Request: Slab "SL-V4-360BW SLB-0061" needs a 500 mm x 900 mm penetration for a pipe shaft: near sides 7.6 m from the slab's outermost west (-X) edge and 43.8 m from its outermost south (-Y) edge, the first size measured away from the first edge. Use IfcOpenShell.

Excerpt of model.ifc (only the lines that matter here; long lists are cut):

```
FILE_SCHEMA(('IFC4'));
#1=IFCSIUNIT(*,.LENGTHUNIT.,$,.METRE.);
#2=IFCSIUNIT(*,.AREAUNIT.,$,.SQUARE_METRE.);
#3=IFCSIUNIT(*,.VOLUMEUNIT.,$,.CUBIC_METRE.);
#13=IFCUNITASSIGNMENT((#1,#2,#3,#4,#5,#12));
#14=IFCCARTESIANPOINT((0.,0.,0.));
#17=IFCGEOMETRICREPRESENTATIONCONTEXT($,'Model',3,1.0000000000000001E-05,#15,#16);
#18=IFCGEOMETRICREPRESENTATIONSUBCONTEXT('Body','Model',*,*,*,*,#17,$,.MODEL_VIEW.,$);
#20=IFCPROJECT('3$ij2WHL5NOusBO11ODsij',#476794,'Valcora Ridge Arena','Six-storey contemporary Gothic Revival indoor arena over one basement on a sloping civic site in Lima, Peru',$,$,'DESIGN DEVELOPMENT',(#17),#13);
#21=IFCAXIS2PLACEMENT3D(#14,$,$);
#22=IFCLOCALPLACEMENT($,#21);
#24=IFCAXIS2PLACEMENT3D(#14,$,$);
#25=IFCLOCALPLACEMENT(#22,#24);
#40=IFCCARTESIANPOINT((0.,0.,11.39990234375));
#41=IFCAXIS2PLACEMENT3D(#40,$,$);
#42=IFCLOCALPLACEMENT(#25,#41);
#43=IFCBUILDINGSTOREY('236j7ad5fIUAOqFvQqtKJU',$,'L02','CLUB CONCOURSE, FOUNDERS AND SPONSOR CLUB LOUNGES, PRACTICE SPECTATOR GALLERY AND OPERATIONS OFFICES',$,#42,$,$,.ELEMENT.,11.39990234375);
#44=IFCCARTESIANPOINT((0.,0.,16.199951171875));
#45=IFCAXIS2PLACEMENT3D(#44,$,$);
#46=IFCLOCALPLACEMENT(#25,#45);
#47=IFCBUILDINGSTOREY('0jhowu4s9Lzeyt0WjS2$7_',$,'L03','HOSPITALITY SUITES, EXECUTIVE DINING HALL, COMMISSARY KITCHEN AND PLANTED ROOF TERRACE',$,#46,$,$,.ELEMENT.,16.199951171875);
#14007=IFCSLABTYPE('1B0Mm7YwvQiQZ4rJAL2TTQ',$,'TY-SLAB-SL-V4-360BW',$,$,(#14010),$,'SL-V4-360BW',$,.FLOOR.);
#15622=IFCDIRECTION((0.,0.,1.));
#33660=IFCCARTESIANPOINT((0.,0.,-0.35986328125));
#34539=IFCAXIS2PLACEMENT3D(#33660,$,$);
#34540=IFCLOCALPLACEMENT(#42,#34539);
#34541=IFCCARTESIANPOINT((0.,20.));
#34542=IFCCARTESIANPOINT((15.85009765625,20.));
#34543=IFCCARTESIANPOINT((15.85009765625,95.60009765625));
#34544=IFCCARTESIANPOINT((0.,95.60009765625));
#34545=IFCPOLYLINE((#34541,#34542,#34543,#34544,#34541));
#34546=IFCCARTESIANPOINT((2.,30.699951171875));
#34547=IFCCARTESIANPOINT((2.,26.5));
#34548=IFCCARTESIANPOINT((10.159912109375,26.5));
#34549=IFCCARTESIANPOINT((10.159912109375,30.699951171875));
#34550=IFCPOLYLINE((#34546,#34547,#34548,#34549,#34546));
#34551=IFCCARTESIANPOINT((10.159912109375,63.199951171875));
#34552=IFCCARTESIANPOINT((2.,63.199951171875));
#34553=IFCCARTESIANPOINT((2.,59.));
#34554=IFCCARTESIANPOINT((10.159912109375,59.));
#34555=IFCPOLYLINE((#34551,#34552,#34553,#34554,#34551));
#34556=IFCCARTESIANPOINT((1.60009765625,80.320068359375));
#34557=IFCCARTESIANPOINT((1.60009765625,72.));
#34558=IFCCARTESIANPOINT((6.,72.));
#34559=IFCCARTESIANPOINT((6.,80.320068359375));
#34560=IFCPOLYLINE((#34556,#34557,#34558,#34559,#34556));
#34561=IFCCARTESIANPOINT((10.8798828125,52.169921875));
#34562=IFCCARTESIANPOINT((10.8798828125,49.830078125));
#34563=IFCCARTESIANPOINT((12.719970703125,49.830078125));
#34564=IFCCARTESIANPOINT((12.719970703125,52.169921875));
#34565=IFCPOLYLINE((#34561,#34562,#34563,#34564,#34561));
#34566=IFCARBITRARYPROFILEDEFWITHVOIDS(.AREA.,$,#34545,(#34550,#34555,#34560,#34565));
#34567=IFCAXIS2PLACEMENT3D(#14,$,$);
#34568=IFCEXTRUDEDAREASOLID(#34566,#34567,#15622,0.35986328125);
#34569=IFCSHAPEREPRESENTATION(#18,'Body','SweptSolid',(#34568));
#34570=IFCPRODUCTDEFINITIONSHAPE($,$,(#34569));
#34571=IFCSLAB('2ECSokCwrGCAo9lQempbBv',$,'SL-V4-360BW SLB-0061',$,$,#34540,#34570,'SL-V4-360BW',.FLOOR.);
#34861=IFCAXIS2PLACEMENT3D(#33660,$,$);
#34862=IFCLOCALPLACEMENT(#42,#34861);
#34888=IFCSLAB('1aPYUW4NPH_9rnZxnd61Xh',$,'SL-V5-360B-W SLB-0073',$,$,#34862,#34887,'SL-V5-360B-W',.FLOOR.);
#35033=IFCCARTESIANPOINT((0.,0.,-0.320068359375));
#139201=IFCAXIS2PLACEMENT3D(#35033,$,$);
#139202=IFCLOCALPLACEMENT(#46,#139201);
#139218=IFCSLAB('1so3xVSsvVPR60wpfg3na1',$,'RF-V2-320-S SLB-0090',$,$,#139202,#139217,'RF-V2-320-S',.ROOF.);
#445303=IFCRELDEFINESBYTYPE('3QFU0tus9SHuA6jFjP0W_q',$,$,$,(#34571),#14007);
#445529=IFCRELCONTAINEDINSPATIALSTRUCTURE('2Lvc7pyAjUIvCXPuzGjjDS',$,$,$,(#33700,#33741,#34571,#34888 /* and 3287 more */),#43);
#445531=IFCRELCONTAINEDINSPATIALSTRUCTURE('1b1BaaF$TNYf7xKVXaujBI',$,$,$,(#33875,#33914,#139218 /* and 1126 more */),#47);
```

```python
import numpy as np
import ifcopenshell
import ifcopenshell.api.feature
import ifcopenshell.api.geometry
import ifcopenshell.api.root
import ifcopenshell.geom
import ifcopenshell.util.placement
import ifcopenshell.util.representation
import ifcopenshell.util.shape
import ifcopenshell.util.unit

model = ifcopenshell.open("model.ifc")
unit_scale = ifcopenshell.util.unit.calculate_unit_scale(model)
settings = ifcopenshell.geom.settings()


def volume(element):
    """Net volume in cubic metres, openings subtracted."""
    shape = ifcopenshell.geom.create_shape(settings, element)
    return ifcopenshell.util.shape.get_volume(shape.geometry)


slab = model.by_guid("2ECSokCwrGCAo9lQempbBv")
before = volume(slab)

# Extent in the slab's own axes, in metres. The edges named are its -X and -Y sides.
slab_shape = ifcopenshell.geom.create_shape(settings, slab)
vertices = ifcopenshell.util.shape.get_vertices(slab_shape.geometry)
x_min, y_min, bottom = vertices.min(axis=0)
top = vertices[:, 2].max()

opening = ifcopenshell.api.root.create_entity(model, ifc_class="IfcOpeningElement", name="Pipe shaft opening", predefined_type="OPENING")
context = ifcopenshell.util.representation.get_context(model, "Model", "Body", "MODEL_VIEW")
width, depth = 0.5, 0.9
outline = [(0.0, 0.0), (width, 0.0), (width, depth), (0.0, depth), (0.0, 0.0)]
# Overshoot both faces by 50 mm so the cut is clean.
shape = ifcopenshell.api.geometry.add_slab_representation(
    model, context=context, depth=top - bottom + 0.1, polyline=outline
)
ifcopenshell.api.geometry.assign_representation(model, product=opening, representation=shape)

matrix = ifcopenshell.util.placement.get_local_placement(slab.ObjectPlacement)
matrix[:, 3] = matrix @ np.append(np.array([x_min + 7.6, y_min + 43.8, bottom - 0.05]) / unit_scale, 1.0)
ifcopenshell.api.geometry.edit_object_placement(model, product=opening, matrix=matrix, is_si=False)
ifcopenshell.api.feature.add_feature(model, feature=opening, element=slab)

after = volume(slab)

print(f"slab volume {before:.3f} -> {after:.3f} m3")

model.write("model-out.ifc")
```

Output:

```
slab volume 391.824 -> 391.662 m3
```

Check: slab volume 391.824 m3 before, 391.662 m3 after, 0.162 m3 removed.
